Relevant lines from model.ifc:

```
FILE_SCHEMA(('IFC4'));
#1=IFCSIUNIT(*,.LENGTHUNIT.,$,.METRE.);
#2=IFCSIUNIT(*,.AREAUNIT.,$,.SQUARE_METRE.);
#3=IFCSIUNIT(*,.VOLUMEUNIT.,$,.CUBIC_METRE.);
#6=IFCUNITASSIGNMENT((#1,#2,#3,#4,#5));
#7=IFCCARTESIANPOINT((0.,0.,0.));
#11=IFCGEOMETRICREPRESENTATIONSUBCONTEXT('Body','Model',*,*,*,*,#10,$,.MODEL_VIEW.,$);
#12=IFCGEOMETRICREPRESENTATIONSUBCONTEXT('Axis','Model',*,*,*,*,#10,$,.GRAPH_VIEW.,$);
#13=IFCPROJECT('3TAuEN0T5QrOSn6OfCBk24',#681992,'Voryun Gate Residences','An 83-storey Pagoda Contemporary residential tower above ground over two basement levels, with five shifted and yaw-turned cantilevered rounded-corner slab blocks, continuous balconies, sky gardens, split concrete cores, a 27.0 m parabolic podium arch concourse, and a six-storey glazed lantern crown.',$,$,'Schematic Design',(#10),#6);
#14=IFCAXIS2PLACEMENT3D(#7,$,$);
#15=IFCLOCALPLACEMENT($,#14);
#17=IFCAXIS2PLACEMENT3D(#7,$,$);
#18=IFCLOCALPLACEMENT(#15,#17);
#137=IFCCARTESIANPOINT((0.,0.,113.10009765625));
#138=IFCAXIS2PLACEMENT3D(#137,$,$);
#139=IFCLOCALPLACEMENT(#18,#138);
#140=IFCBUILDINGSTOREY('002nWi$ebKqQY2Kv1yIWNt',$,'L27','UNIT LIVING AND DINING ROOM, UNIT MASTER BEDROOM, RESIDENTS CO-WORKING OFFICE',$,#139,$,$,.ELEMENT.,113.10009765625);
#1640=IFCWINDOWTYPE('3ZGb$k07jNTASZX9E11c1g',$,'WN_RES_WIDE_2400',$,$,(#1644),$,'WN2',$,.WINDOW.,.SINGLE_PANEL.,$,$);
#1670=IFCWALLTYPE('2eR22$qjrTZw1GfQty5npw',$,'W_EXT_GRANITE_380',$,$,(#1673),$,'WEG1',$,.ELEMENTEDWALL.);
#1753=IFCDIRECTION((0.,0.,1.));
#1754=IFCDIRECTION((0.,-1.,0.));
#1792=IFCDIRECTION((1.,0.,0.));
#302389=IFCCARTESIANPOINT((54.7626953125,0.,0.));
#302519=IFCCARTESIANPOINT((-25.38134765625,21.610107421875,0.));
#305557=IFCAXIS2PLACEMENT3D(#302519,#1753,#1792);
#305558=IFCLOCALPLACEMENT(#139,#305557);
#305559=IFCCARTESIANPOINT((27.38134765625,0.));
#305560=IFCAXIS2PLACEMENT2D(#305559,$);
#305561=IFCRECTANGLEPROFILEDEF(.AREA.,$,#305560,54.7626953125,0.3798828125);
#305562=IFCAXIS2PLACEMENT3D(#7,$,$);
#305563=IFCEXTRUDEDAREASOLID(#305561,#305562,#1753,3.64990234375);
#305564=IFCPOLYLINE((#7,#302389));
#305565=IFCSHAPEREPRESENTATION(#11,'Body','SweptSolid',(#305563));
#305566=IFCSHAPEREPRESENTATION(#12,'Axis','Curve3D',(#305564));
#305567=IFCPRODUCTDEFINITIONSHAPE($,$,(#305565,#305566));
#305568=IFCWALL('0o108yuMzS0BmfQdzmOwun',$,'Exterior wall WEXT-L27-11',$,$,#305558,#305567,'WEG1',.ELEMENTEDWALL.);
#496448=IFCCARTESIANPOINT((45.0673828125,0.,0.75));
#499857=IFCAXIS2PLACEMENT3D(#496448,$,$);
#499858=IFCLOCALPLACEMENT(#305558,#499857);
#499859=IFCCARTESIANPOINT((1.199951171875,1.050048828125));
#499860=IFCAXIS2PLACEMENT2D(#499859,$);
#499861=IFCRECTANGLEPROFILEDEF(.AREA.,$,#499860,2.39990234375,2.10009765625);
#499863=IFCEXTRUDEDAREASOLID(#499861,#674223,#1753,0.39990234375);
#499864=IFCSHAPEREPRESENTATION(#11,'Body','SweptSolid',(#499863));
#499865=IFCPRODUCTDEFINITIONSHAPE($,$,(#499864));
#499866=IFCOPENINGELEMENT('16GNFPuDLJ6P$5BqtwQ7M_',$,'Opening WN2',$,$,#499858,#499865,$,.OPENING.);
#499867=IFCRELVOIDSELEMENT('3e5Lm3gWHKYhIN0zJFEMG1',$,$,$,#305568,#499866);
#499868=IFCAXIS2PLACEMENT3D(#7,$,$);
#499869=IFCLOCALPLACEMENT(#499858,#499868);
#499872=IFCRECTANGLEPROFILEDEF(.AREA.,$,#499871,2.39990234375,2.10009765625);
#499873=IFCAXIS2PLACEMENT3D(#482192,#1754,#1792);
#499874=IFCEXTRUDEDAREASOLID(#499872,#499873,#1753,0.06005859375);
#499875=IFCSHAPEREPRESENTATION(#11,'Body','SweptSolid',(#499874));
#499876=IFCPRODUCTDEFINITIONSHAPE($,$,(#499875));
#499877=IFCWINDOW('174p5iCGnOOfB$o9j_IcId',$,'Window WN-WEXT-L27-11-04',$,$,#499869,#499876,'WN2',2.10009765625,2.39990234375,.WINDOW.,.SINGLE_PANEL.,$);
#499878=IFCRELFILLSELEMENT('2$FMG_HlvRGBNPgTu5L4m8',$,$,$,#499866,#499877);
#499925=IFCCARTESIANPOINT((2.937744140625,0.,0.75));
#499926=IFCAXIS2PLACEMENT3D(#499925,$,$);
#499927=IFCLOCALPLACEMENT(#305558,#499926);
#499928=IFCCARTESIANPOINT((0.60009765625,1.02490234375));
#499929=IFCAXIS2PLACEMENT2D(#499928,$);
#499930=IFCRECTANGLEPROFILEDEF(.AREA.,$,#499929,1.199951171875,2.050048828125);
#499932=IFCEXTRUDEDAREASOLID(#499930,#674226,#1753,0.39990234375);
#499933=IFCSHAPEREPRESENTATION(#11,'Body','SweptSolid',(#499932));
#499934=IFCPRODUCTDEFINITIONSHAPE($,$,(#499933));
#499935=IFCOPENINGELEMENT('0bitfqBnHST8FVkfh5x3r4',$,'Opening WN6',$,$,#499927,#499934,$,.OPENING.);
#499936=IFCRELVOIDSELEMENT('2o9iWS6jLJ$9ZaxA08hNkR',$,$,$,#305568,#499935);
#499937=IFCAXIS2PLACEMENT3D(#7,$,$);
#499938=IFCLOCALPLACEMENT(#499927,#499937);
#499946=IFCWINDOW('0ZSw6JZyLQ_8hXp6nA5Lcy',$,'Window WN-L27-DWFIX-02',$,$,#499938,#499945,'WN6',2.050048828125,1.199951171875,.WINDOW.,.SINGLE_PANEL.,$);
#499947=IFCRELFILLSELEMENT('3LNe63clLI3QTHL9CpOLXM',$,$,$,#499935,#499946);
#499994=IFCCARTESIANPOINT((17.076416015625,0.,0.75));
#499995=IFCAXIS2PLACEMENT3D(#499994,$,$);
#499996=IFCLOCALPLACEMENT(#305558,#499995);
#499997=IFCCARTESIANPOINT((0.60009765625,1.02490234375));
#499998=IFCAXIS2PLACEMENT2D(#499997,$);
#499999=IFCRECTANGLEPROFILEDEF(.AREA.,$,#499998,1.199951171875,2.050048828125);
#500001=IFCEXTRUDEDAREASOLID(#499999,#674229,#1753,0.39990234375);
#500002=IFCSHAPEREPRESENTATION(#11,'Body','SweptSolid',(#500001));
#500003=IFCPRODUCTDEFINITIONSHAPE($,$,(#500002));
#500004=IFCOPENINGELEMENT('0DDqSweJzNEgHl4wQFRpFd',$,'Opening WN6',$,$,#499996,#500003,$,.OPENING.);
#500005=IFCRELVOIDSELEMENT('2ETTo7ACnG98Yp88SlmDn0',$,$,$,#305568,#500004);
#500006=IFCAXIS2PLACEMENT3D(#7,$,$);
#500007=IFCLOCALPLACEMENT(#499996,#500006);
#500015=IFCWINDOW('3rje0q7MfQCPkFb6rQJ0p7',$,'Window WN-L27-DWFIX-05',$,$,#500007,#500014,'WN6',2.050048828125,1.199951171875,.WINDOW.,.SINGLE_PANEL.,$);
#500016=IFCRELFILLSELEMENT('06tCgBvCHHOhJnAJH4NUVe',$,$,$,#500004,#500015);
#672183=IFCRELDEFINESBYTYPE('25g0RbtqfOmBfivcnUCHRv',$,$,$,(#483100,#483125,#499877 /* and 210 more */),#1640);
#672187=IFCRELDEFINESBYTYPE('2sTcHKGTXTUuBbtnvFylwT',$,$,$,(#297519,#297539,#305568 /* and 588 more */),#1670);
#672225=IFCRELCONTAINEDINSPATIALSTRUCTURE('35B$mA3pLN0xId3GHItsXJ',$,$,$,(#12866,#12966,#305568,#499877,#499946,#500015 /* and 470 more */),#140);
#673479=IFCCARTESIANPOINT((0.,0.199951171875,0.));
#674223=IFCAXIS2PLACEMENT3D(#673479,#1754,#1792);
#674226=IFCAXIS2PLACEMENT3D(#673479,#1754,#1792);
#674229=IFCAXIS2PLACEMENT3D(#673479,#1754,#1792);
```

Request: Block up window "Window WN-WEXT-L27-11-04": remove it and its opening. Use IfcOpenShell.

```python
import ifcopenshell
import ifcopenshell.api.feature
import ifcopenshell.api.root
import ifcopenshell.geom
import ifcopenshell.util.shape

model = ifcopenshell.open("model.ifc")
settings = ifcopenshell.geom.settings()


def volume(element):
    """Net volume in cubic metres, openings subtracted."""
    shape = ifcopenshell.geom.create_shape(settings, element)
    return ifcopenshell.util.shape.get_volume(shape.geometry)


window = model.by_guid("174p5iCGnOOfB$o9j_IcId")
opening = window.FillsVoids[0].RelatingOpeningElement
wall = opening.VoidsElements[0].RelatingBuildingElement
before = volume(wall)

ifcopenshell.api.root.remove_product(model, product=window)
ifcopenshell.api.feature.remove_feature(model, feature=opening)

after = volume(wall)

print(f"wall volume {before:.3f} -> {after:.3f} m3")

model.write("model_rev.ifc")
```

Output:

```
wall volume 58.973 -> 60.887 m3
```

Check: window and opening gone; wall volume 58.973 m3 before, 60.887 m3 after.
